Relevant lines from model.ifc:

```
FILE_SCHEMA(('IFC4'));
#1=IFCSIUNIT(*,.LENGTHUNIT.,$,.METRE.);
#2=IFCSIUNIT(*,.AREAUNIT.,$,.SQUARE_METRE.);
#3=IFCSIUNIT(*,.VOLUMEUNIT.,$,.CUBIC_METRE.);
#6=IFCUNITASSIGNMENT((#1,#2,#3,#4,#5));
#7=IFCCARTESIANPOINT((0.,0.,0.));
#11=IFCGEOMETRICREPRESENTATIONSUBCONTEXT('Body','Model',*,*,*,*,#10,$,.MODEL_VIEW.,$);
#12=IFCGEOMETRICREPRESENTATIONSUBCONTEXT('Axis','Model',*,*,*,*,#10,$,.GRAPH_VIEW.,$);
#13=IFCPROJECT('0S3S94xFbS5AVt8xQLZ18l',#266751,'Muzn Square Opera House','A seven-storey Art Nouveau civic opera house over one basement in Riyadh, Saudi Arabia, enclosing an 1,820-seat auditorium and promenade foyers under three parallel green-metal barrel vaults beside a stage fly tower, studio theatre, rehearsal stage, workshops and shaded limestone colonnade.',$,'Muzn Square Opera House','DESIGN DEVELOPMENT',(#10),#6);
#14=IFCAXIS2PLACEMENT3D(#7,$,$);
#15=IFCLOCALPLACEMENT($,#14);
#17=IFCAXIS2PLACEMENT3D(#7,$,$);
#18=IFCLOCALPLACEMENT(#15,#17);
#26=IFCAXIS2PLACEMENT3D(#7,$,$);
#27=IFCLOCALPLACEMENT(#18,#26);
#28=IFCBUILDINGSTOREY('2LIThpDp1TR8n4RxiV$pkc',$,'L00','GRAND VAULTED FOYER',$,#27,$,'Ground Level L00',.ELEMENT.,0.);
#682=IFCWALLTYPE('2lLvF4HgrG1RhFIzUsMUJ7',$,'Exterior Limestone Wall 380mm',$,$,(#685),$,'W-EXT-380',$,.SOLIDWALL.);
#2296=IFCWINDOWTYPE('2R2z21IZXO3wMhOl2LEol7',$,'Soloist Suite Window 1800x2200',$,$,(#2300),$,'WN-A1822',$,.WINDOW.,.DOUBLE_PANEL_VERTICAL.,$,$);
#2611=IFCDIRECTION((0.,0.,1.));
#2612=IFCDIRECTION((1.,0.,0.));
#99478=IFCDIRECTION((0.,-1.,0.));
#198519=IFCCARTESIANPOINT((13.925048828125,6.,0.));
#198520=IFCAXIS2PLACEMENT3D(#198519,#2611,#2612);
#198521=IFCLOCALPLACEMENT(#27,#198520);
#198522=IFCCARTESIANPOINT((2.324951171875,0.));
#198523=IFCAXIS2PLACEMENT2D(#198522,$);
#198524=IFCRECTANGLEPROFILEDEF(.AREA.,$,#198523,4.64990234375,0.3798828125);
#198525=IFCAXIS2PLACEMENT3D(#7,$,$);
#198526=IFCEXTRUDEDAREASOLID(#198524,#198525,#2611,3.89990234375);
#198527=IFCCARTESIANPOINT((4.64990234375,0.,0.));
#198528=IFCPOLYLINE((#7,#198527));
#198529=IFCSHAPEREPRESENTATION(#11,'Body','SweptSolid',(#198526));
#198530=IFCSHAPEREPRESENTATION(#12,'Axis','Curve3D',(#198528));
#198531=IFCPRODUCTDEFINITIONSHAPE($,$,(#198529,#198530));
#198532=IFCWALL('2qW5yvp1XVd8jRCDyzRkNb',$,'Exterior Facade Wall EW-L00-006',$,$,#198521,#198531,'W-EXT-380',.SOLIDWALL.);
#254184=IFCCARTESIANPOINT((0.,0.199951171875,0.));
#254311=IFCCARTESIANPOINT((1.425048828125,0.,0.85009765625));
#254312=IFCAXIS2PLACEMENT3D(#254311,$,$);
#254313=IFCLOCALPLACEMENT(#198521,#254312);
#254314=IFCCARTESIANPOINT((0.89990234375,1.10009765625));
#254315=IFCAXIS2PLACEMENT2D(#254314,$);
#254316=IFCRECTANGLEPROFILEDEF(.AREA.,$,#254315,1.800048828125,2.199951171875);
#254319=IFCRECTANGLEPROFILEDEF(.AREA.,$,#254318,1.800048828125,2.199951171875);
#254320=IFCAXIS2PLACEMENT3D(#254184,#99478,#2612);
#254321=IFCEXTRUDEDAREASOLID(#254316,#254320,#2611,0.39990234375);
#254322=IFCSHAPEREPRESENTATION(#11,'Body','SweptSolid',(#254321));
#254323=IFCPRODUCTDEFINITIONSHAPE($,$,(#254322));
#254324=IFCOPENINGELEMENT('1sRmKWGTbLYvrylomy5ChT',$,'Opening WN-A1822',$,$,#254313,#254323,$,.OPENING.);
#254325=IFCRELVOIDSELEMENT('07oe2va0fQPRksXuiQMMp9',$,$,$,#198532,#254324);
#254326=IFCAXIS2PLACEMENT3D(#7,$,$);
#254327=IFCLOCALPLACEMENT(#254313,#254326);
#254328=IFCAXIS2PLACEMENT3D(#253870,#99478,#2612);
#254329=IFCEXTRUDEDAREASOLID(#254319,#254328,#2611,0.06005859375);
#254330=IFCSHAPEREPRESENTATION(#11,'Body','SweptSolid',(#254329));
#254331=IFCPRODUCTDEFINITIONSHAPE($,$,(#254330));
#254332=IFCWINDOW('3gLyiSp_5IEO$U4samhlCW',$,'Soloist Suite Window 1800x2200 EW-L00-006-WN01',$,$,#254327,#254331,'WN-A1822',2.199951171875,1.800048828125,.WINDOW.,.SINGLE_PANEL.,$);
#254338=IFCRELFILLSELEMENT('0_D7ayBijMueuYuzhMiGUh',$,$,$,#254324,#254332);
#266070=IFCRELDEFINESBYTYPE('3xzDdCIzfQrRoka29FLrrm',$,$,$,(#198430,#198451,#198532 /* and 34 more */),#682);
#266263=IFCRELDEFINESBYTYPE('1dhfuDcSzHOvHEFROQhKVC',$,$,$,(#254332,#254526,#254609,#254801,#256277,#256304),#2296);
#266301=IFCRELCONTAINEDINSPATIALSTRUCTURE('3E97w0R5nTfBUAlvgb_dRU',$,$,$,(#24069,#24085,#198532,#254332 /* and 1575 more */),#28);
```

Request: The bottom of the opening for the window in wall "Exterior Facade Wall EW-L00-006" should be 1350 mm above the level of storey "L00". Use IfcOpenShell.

```python
import numpy as np
import ifcopenshell
import ifcopenshell.api.geometry
import ifcopenshell.geom
import ifcopenshell.util.element
import ifcopenshell.util.placement
import ifcopenshell.util.shape
import ifcopenshell.util.unit

model = ifcopenshell.open("model.ifc")
unit_scale = ifcopenshell.util.unit.calculate_unit_scale(model)

window = model.by_id(254332)
opening = window.FillsVoids[0].RelatingOpeningElement
storey = ifcopenshell.util.element.get_container(window, ifc_class="IfcBuildingStorey")
level = ifcopenshell.util.placement.get_local_placement(storey.ObjectPlacement)[2, 3]

# The opening's origin need not be at the sill, so measure its lowest point.
shape = ifcopenshell.geom.create_shape(ifcopenshell.geom.settings(), opening)
bottom = ifcopenshell.util.shape.get_shape_bottom_elevation(shape, shape.geometry) / unit_scale
dz = level + 1.35 / unit_scale - bottom

shift = np.array([0.0, 0.0, dz])
# The window is placed relative to its opening, so it follows when the opening moves.
matrix = ifcopenshell.util.placement.get_local_placement(opening.ObjectPlacement)
matrix[:3, 3] += shift
ifcopenshell.api.geometry.edit_object_placement(
    model, product=opening, matrix=matrix, is_si=False, should_transform_children=True
)

print(f"moved by {dz * unit_scale:+.3f} m")

model.write("model-out.ifc")
```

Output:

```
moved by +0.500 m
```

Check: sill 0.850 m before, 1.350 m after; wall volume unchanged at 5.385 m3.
